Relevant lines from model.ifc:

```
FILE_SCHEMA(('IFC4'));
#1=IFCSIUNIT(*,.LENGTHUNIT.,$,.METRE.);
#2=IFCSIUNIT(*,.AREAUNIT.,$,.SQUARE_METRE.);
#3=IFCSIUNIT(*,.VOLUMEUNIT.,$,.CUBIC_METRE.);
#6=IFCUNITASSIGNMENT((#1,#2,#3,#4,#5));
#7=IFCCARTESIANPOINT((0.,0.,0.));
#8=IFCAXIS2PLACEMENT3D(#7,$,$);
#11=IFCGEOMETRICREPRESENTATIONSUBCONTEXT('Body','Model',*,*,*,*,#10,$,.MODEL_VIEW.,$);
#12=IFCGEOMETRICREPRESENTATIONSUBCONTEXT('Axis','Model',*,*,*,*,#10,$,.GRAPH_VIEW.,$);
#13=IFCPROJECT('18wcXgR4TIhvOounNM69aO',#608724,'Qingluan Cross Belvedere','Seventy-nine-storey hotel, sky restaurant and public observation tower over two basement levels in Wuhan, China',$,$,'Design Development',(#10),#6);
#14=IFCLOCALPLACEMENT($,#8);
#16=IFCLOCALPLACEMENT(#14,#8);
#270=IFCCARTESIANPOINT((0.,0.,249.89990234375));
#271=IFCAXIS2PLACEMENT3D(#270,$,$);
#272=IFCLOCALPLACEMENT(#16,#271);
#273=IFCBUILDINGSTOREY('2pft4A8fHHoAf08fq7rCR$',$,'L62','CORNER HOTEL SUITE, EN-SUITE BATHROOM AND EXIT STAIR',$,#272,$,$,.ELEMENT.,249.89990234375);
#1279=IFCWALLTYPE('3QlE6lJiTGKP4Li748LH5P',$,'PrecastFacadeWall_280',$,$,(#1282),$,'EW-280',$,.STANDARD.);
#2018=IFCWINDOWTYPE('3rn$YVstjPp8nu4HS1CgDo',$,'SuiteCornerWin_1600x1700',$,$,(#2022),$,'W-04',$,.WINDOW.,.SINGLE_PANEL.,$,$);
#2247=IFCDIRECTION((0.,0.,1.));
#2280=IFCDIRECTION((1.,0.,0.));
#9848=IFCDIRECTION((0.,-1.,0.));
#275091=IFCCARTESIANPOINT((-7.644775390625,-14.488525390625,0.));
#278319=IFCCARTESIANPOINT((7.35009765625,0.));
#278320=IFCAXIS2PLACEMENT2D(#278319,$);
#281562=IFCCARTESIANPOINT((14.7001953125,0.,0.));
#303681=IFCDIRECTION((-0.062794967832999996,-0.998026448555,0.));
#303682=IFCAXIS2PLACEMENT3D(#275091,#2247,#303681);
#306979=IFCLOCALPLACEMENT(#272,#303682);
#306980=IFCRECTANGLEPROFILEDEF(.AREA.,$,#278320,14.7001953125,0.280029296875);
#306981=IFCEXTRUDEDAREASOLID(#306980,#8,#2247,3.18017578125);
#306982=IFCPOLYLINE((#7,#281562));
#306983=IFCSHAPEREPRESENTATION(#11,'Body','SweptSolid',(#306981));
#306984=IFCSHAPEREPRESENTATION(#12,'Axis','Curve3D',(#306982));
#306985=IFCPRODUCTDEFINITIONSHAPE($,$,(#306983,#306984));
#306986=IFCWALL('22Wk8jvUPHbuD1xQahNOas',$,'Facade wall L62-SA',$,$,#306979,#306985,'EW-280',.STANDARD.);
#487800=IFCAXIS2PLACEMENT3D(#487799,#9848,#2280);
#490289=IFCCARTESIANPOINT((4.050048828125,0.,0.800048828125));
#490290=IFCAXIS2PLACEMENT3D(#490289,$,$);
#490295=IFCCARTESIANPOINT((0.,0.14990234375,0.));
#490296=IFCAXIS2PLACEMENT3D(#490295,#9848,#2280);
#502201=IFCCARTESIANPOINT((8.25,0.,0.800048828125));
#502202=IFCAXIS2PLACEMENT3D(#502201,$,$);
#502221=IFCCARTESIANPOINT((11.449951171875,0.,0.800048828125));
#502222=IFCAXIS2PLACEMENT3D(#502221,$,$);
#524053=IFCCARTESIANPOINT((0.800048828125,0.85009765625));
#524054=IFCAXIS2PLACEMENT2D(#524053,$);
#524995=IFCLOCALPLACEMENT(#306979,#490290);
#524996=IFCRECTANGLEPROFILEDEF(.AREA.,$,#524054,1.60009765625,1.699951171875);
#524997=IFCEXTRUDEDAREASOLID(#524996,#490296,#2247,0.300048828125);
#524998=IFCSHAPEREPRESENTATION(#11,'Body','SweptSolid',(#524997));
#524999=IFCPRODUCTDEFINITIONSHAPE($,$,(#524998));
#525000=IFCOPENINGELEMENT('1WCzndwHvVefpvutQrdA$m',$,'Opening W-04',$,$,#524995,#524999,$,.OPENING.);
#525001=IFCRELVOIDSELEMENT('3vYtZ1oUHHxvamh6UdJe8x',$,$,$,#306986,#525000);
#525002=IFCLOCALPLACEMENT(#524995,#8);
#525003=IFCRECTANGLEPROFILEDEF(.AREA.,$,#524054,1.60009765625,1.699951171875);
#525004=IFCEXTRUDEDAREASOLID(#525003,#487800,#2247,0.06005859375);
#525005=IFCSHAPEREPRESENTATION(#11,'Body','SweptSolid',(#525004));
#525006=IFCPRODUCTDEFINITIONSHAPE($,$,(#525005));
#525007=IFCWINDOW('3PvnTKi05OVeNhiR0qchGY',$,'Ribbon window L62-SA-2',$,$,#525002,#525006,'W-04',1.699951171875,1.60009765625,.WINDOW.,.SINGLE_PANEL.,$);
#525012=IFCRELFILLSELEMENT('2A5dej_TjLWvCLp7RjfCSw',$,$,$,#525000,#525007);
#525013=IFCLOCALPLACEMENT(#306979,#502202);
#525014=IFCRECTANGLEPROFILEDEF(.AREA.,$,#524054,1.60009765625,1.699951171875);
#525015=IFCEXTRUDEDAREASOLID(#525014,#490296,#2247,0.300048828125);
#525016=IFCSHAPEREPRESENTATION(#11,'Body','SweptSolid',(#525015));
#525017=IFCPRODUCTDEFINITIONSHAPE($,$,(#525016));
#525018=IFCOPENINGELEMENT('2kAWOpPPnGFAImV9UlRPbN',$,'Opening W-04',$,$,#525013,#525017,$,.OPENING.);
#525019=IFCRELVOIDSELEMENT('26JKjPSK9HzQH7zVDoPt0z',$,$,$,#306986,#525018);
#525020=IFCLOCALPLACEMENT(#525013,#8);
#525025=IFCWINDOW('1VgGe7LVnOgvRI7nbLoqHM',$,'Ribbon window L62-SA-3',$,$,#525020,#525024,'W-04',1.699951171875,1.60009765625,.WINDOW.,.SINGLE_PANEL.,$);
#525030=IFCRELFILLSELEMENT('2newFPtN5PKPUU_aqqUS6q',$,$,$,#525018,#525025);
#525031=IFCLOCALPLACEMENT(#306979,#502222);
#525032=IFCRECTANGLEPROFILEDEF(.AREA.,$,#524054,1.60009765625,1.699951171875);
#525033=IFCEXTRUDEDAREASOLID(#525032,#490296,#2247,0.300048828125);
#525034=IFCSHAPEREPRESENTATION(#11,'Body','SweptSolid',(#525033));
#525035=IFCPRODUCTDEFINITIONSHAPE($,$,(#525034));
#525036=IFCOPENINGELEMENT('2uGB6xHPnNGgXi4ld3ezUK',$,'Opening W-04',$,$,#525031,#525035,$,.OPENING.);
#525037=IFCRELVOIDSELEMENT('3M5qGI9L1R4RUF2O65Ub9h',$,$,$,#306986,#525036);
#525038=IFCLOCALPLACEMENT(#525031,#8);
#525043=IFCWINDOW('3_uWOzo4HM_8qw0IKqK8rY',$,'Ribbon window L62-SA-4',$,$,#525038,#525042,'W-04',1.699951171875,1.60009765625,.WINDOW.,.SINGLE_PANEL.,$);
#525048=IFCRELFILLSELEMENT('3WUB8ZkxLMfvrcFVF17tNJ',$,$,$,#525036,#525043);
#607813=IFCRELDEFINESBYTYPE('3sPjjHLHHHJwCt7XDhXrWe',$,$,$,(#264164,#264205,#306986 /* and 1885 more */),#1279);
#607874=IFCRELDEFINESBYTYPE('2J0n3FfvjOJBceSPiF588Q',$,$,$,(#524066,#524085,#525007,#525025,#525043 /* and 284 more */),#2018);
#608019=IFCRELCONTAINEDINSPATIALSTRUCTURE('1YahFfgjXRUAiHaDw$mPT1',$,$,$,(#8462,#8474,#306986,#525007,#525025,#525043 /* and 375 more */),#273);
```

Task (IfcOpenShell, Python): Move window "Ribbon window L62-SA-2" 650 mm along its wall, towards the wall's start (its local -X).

```python
import ifcopenshell
import ifcopenshell.api.geometry
import ifcopenshell.util.placement

model = ifcopenshell.open("model.ifc")

window = model.by_id(525007)
opening = window.FillsVoids[0].RelatingOpeningElement
wall = opening.VoidsElements[0].RelatingBuildingElement

wall_matrix = ifcopenshell.util.placement.get_local_placement(wall.ObjectPlacement)
shift = wall_matrix[:3, 0] * -0.65
before = ifcopenshell.util.placement.get_local_placement(window.ObjectPlacement)[:3, 3].copy()

# The window is placed relative to its opening, so it follows when the opening moves.
matrix = ifcopenshell.util.placement.get_local_placement(opening.ObjectPlacement)
matrix[:3, 3] += shift
ifcopenshell.api.geometry.edit_object_placement(
    model, product=opening, matrix=matrix, is_si=False, should_transform_children=True
)

after = ifcopenshell.util.placement.get_local_placement(window.ObjectPlacement)[:3, 3]
print("window moved by", (after - before).round(3) + 0.0)

model.write("model_updated.ifc")
```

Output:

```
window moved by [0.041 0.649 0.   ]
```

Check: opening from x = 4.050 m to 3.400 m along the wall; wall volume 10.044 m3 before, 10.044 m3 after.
